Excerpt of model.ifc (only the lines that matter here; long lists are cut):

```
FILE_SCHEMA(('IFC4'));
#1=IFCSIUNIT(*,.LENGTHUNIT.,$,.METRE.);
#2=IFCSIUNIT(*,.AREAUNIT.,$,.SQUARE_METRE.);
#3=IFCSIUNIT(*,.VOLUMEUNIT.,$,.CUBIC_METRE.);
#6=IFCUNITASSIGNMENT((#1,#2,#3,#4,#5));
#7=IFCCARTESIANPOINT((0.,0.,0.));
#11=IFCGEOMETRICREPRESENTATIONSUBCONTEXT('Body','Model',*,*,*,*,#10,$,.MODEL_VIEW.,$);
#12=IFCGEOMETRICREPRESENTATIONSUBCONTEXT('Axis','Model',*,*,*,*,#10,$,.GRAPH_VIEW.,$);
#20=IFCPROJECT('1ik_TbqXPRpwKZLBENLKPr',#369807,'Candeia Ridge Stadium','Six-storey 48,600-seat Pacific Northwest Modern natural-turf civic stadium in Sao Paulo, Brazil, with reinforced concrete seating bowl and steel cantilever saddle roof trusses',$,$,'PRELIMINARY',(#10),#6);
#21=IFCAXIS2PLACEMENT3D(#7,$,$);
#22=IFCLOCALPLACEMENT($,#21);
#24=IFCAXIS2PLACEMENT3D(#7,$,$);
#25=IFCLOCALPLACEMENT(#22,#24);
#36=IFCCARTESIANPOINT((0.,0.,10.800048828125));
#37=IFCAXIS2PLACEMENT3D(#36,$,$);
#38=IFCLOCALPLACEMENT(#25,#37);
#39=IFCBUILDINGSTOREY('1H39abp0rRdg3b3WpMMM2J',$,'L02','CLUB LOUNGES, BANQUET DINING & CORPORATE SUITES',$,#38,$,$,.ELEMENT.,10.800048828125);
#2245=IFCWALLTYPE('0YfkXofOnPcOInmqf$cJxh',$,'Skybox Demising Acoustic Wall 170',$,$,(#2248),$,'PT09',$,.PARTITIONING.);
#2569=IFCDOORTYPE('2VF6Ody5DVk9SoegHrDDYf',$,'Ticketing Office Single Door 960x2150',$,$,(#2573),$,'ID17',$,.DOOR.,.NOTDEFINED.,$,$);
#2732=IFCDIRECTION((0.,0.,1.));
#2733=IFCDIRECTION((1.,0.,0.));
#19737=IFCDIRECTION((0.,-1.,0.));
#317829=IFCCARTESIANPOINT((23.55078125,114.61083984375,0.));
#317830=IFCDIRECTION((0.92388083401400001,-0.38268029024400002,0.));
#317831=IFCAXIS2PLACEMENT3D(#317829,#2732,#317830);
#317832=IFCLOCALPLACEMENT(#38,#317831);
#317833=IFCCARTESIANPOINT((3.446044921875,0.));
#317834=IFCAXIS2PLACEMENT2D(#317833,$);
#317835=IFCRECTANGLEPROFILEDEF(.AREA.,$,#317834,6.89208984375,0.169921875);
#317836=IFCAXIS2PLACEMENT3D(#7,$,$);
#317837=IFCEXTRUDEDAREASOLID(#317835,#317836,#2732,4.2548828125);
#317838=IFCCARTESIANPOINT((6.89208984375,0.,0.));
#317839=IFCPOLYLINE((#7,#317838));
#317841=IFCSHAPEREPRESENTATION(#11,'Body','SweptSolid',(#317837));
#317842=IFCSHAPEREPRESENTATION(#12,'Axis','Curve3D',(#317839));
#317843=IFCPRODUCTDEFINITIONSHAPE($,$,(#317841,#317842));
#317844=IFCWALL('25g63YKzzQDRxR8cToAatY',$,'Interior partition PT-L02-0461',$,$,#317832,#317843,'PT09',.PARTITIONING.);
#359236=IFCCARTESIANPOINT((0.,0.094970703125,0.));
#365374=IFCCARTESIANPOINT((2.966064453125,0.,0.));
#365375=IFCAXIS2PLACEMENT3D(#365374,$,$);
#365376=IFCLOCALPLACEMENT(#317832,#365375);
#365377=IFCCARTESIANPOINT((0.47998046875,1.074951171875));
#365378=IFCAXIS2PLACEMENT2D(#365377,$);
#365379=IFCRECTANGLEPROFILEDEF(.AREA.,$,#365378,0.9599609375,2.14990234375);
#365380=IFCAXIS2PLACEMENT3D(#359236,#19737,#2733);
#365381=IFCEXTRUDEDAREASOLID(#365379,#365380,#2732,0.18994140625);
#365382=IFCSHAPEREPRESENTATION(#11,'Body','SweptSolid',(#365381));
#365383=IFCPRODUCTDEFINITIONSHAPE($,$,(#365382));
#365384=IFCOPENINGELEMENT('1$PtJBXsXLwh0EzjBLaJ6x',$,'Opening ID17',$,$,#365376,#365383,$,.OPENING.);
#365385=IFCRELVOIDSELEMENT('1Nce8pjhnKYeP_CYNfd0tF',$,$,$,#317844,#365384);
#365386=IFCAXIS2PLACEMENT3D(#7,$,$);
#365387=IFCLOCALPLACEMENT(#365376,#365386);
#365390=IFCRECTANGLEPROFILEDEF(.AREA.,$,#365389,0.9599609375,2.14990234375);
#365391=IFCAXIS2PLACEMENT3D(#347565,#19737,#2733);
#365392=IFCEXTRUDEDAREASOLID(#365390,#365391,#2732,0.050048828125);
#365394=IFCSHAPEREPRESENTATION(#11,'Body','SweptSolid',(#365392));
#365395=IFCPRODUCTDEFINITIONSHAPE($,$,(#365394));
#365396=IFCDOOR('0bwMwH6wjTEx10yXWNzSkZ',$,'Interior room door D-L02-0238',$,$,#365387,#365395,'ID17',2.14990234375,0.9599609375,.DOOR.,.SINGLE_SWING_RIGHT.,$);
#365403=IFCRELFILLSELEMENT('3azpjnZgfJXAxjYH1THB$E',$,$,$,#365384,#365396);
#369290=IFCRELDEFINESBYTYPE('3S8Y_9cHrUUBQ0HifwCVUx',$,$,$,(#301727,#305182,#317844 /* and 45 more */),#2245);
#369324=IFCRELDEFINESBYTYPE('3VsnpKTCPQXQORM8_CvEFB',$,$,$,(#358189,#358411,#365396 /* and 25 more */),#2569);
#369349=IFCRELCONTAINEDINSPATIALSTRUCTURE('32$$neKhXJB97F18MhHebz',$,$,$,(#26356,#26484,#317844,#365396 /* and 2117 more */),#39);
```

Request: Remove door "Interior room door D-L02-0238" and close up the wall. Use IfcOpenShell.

```python
import ifcopenshell
import ifcopenshell.api.feature
import ifcopenshell.api.root
import ifcopenshell.geom
import ifcopenshell.util.shape

model = ifcopenshell.open("model.ifc")
settings = ifcopenshell.geom.settings()


def volume(element):
    """Net volume in cubic metres, openings subtracted."""
    shape = ifcopenshell.geom.create_shape(settings, element)
    return ifcopenshell.util.shape.get_volume(shape.geometry)


door = model.by_guid("0bwMwH6wjTEx10yXWNzSkZ")
opening = door.FillsVoids[0].RelatingOpeningElement
wall = opening.VoidsElements[0].RelatingBuildingElement
before = volume(wall)

ifcopenshell.api.root.remove_product(model, product=door)
ifcopenshell.api.feature.remove_feature(model, feature=opening)

after = volume(wall)

print(f"wall volume {before:.3f} -> {after:.3f} m3")

model.write("model_edited.ifc")
```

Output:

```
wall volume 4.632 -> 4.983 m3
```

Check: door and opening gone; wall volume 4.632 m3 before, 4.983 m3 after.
